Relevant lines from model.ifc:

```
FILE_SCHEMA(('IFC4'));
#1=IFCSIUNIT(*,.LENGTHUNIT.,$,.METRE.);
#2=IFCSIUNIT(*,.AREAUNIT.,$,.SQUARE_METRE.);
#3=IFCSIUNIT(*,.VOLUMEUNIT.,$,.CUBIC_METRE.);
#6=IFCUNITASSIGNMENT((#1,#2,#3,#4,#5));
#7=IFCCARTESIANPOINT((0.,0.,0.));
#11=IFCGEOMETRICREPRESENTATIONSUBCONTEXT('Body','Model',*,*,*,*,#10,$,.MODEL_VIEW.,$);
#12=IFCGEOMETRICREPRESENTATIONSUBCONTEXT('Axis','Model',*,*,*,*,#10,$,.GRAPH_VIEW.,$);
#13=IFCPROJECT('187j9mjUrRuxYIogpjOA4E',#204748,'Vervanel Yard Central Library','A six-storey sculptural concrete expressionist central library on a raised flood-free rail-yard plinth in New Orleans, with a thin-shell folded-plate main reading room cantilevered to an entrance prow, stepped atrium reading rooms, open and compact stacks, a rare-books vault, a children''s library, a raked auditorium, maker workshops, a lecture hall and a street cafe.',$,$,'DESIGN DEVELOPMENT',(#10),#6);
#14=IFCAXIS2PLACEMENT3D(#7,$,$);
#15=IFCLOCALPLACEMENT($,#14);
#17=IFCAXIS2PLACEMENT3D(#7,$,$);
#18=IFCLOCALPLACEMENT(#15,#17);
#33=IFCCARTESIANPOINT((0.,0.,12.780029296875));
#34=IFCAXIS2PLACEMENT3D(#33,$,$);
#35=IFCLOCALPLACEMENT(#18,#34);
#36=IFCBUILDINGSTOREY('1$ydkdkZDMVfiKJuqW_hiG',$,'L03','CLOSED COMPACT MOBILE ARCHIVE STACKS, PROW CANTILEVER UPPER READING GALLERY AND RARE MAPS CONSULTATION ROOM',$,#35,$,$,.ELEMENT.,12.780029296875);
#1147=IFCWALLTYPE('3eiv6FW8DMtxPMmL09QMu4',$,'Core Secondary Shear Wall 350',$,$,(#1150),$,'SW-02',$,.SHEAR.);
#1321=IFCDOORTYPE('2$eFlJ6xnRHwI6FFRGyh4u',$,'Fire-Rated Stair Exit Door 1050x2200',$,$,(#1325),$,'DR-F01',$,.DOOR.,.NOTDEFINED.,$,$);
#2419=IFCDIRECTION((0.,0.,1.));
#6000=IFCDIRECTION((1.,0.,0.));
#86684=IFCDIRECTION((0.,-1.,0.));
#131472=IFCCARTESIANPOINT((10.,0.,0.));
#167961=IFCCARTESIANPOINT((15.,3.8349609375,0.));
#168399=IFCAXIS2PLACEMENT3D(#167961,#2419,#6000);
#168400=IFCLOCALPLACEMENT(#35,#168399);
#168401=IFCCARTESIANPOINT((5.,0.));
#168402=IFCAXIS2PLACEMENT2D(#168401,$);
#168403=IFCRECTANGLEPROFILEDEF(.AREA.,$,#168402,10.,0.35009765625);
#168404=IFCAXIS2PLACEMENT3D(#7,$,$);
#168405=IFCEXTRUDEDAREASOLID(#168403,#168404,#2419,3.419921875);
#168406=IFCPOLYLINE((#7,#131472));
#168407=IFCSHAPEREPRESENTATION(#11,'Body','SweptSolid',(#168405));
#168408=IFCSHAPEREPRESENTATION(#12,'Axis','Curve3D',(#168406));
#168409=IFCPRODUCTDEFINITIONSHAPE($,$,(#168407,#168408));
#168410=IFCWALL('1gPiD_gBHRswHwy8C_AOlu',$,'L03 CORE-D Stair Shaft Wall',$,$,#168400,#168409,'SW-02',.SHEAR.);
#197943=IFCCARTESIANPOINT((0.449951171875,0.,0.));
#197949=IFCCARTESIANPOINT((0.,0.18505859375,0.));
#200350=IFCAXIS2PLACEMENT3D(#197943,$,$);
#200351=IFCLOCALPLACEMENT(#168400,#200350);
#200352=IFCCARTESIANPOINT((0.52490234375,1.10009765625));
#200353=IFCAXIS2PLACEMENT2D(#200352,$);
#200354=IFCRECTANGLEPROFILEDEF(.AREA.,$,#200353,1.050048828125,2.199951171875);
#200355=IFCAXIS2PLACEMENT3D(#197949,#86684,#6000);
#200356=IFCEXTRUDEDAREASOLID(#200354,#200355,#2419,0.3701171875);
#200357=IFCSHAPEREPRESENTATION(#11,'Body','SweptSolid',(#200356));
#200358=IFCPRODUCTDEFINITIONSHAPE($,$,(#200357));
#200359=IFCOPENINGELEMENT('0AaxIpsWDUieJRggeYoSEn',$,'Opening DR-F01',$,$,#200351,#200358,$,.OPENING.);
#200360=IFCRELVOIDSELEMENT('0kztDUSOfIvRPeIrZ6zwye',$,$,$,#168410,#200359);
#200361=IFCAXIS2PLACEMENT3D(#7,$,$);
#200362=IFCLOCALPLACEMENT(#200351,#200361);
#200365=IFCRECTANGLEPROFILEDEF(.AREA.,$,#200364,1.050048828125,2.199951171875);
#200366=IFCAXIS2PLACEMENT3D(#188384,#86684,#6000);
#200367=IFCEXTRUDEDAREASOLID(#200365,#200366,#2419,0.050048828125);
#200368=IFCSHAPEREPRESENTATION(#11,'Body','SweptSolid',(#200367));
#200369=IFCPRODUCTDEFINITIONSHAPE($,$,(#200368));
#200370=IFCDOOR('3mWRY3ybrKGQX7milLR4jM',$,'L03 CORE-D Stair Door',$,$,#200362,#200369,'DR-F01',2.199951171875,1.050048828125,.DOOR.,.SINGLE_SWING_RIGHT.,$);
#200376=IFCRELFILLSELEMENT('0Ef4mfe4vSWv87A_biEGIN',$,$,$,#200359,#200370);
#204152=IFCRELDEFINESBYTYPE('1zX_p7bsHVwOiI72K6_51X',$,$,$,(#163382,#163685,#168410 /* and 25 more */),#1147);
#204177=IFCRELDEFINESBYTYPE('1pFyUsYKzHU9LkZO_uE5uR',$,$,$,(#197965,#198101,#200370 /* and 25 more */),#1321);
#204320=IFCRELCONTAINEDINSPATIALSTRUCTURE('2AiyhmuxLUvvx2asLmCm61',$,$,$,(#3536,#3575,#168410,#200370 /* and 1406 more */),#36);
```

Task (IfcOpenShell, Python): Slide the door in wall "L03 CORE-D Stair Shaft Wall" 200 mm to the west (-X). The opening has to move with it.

```python
import ifcopenshell
import ifcopenshell.api.geometry
import ifcopenshell.util.placement
import ifcopenshell.util.unit

model = ifcopenshell.open("model.ifc")
unit_scale = ifcopenshell.util.unit.calculate_unit_scale(model)

door = model.by_guid("3mWRY3ybrKGQX7milLR4jM")
opening = door.FillsVoids[0].RelatingOpeningElement
wall = opening.VoidsElements[0].RelatingBuildingElement

wall_matrix = ifcopenshell.util.placement.get_local_placement(wall.ObjectPlacement)
shift = wall_matrix[:3, 0] * -0.2 / unit_scale
before = ifcopenshell.util.placement.get_local_placement(door.ObjectPlacement)[:3, 3].copy()

# The door is placed relative to its opening, so it follows when the opening moves.
matrix = ifcopenshell.util.placement.get_local_placement(opening.ObjectPlacement)
matrix[:3, 3] += shift
ifcopenshell.api.geometry.edit_object_placement(
    model, product=opening, matrix=matrix, is_si=False, should_transform_children=True
)

after = ifcopenshell.util.placement.get_local_placement(door.ObjectPlacement)[:3, 3]
print("door moved by", (after - before).round(3) + 0.0)

model.write("model_rev.ifc")
```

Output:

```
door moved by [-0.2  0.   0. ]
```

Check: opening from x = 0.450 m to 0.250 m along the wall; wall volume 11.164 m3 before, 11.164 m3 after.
